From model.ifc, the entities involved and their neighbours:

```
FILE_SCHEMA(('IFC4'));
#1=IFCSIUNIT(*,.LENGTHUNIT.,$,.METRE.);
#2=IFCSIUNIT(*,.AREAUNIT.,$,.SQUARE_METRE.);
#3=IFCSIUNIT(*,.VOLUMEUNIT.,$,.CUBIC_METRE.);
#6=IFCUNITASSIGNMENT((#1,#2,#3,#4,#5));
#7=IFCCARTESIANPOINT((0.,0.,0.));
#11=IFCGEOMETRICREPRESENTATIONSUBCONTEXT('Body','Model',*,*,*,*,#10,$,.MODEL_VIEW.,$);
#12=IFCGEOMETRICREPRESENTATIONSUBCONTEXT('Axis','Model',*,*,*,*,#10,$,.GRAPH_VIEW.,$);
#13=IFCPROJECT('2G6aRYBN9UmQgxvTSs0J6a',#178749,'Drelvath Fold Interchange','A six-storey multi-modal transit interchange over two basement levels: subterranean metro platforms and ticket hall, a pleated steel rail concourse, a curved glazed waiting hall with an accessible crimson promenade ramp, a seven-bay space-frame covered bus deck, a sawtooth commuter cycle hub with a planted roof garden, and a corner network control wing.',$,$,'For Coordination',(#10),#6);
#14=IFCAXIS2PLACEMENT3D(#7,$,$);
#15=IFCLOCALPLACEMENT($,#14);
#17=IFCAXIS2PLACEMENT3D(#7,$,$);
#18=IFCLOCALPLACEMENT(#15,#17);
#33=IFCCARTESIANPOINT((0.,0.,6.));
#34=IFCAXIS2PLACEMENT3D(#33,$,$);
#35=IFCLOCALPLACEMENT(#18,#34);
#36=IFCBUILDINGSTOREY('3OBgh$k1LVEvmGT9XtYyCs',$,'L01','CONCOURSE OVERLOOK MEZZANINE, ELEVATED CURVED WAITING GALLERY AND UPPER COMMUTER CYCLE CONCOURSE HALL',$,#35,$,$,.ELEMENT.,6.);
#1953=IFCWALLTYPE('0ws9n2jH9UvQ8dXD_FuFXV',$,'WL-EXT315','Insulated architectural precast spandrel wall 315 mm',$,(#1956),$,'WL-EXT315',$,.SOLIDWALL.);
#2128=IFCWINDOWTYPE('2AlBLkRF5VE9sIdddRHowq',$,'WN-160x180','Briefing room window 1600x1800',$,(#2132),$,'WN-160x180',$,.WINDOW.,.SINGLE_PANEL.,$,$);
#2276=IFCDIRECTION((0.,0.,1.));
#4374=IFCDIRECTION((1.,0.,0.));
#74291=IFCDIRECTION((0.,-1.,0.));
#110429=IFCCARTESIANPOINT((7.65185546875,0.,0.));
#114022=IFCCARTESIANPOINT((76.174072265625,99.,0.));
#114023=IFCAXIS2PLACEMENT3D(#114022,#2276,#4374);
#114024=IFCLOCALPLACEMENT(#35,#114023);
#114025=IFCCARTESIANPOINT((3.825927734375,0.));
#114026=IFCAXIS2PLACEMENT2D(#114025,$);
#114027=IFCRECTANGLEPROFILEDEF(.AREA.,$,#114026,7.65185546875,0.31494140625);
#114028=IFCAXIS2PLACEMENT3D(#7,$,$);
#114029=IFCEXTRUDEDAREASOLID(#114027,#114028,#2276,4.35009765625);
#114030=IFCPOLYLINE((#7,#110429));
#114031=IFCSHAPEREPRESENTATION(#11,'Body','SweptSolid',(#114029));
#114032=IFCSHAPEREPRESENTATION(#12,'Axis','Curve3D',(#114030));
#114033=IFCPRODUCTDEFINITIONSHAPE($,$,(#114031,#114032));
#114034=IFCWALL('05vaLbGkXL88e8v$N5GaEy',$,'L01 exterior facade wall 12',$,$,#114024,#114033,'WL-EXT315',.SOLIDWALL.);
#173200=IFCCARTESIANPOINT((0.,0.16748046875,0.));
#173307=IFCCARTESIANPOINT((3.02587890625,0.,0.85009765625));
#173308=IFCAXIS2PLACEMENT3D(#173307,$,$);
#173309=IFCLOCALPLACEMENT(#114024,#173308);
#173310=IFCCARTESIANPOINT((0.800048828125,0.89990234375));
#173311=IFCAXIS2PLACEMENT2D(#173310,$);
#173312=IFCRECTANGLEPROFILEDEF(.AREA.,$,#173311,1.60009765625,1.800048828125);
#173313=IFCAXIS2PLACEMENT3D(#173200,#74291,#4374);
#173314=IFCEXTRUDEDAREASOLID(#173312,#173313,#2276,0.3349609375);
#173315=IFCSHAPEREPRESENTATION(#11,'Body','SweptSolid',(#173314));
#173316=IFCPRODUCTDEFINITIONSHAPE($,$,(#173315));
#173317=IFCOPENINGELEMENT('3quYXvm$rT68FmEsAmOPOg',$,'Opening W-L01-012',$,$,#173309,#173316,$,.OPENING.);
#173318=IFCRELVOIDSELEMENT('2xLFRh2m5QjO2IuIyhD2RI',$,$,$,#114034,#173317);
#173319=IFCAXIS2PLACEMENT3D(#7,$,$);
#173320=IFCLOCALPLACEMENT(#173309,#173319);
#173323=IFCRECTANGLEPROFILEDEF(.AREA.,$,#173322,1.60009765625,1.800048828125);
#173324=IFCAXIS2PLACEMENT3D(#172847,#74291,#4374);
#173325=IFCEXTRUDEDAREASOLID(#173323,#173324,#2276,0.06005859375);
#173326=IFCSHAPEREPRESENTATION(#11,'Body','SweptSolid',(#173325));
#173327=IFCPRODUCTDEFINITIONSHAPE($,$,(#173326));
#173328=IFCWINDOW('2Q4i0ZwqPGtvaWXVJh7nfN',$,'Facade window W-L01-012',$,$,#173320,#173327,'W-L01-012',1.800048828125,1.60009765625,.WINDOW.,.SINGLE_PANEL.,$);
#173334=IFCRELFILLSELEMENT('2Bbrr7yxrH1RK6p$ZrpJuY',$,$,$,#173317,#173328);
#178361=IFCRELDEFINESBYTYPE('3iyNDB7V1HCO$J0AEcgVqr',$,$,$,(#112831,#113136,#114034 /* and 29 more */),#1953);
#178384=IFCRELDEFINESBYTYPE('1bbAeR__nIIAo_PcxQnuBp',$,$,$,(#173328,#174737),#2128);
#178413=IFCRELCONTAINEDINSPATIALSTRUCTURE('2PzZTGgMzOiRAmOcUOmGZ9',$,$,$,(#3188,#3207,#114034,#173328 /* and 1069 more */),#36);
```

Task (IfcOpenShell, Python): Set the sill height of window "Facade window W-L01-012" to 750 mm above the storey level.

```python
import numpy as np
import ifcopenshell
import ifcopenshell.api.geometry
import ifcopenshell.geom
import ifcopenshell.util.element
import ifcopenshell.util.placement
import ifcopenshell.util.shape
import ifcopenshell.util.unit

model = ifcopenshell.open("model.ifc")
unit_scale = ifcopenshell.util.unit.calculate_unit_scale(model)

window = model.by_id(173328)
opening = window.FillsVoids[0].RelatingOpeningElement
storey = ifcopenshell.util.element.get_container(window, ifc_class="IfcBuildingStorey")
level = ifcopenshell.util.placement.get_local_placement(storey.ObjectPlacement)[2, 3]

# The opening's origin need not be at the sill, so measure its lowest point.
shape = ifcopenshell.geom.create_shape(ifcopenshell.geom.settings(), opening)
bottom = ifcopenshell.util.shape.get_shape_bottom_elevation(shape, shape.geometry) / unit_scale
dz = level + 0.75 / unit_scale - bottom

shift = np.array([0.0, 0.0, dz])
# The window is placed relative to its opening, so it follows when the opening moves.
matrix = ifcopenshell.util.placement.get_local_placement(opening.ObjectPlacement)
matrix[:3, 3] += shift
ifcopenshell.api.geometry.edit_object_placement(
    model, product=opening, matrix=matrix, is_si=False, should_transform_children=True
)

print(f"moved by {dz * unit_scale:+.3f} m")

model.write("model_v2.ifc")
```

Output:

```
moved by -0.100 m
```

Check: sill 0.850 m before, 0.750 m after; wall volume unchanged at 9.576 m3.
